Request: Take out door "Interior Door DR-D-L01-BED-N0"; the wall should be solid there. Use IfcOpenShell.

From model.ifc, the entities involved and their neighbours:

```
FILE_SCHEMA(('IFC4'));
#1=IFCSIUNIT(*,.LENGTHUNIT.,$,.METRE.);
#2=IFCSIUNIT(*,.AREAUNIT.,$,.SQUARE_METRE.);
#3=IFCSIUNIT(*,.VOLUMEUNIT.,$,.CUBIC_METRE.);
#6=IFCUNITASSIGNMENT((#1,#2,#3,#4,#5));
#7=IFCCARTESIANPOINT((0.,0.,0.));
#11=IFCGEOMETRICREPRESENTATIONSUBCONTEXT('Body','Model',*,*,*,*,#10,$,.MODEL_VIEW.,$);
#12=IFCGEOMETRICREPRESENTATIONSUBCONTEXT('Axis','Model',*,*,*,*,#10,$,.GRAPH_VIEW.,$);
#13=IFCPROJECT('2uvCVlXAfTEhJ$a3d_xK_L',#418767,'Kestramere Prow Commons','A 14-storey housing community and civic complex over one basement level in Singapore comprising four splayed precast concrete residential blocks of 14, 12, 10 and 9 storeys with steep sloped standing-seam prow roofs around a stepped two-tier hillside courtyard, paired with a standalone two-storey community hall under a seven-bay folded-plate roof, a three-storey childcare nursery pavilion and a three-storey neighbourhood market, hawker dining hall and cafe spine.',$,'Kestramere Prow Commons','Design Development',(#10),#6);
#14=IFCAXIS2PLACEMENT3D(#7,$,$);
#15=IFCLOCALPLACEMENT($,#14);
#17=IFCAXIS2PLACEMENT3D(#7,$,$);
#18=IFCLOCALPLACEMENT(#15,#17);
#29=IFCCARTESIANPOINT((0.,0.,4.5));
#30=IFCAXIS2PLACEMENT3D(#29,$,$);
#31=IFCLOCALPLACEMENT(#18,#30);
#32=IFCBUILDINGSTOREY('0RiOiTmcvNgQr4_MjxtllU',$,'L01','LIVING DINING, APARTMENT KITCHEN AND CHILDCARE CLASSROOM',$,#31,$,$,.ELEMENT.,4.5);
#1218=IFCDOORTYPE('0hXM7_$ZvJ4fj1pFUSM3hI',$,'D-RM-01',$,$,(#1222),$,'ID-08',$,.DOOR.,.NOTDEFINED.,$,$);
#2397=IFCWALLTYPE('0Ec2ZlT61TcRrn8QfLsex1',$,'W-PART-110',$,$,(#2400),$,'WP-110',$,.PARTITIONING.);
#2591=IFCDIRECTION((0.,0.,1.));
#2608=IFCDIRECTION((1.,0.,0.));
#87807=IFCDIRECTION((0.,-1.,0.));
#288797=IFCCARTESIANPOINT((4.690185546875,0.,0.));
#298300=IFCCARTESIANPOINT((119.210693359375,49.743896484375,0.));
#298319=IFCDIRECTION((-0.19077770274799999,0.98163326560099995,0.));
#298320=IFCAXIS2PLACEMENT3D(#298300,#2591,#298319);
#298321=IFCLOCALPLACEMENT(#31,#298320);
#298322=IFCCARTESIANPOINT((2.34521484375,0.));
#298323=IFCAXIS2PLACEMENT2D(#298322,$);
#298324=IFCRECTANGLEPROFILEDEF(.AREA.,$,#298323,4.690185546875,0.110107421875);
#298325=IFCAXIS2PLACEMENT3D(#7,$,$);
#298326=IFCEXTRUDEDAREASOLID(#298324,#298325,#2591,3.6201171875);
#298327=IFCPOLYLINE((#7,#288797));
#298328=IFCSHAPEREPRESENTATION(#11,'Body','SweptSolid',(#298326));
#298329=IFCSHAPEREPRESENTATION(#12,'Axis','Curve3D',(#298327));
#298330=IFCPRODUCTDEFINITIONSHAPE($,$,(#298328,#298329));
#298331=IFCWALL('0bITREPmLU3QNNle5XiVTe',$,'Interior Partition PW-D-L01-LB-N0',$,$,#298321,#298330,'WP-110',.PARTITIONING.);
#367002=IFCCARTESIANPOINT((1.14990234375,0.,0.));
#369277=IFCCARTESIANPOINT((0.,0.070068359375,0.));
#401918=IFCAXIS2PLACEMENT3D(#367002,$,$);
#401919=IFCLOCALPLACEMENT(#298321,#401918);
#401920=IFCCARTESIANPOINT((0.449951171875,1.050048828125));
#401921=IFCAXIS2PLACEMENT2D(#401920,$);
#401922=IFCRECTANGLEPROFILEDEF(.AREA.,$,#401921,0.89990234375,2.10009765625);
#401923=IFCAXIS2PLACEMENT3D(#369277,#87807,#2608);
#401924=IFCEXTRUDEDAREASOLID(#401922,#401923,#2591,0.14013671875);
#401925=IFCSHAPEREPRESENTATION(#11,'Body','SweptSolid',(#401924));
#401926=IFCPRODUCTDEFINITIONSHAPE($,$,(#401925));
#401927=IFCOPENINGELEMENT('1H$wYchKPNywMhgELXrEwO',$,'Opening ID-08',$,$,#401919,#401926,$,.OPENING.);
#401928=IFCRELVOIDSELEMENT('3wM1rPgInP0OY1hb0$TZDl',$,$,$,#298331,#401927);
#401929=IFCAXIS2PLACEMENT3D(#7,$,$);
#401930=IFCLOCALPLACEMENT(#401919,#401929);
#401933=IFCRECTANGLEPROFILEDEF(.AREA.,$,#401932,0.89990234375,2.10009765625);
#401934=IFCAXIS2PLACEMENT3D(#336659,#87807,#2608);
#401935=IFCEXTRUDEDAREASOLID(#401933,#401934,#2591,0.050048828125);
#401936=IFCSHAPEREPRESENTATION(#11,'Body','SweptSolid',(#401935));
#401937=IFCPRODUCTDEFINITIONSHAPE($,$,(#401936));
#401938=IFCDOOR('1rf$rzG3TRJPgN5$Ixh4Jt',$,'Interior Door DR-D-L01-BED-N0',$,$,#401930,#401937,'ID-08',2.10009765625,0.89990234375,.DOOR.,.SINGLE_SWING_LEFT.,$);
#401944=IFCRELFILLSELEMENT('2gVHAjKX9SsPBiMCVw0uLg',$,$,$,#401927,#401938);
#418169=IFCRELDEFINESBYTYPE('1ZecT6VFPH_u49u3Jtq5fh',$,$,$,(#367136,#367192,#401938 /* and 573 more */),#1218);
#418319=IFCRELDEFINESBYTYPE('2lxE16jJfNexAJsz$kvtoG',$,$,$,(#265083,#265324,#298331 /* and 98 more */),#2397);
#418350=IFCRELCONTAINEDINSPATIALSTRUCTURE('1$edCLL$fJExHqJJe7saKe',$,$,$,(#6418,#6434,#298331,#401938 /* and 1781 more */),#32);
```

```python
import ifcopenshell
import ifcopenshell.api.feature
import ifcopenshell.api.root
import ifcopenshell.geom
import ifcopenshell.util.shape

model = ifcopenshell.open("model.ifc")
settings = ifcopenshell.geom.settings()


def volume(element):
    """Net volume in cubic metres, openings subtracted."""
    shape = ifcopenshell.geom.create_shape(settings, element)
    return ifcopenshell.util.shape.get_volume(shape.geometry)


door = model.by_guid("1rf$rzG3TRJPgN5$Ixh4Jt")
opening = door.FillsVoids[0].RelatingOpeningElement
wall = opening.VoidsElements[0].RelatingBuildingElement
before = volume(wall)

ifcopenshell.api.root.remove_product(model, product=door)
ifcopenshell.api.feature.remove_feature(model, feature=opening)

after = volume(wall)

print(f"wall volume {before:.3f} -> {after:.3f} m3")

model.write("model_updated.ifc")
```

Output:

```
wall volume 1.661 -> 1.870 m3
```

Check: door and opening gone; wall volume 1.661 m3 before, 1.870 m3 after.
